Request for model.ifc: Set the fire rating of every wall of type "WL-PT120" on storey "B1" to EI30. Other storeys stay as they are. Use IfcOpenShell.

First a look at what the model holds.

```python
import ifcopenshell
import ifcopenshell.util.element

model = ifcopenshell.open("model.ifc")
print(model.schema)
storey = next(s for s in model.by_type("IfcBuildingStorey") if s.Name == "B1")
walls = [e for e in ifcopenshell.util.element.get_decomposition(storey) if e.is_a("IfcWall")]
seen = {}
for e in walls:
    element_type = ifcopenshell.util.element.get_type(e)
    key = (element_type.Name if element_type != e and element_type else None, ifcopenshell.util.element.get_pset(e, "Pset_WallCommon", "FireRating"))
    seen[key] = seen.get(key, 0) + 1
for (name, value), count in sorted(seen.items(), key=str):
    print(count, "x", name, "|", value)
```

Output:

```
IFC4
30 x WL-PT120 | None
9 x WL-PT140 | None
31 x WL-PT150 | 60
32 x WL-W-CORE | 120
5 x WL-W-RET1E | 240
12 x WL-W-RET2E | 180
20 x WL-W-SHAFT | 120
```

```python
import ifcopenshell
import ifcopenshell.api.pset
import ifcopenshell.util.element

model = ifcopenshell.open("model.ifc")

storey = next(s for s in model.by_type("IfcBuildingStorey") if s.Name == "B1")
walls = [e for e in ifcopenshell.util.element.get_decomposition(storey) if e.is_a("IfcWall")]

count = 0
for e in walls:
    element_type = ifcopenshell.util.element.get_type(e)
    if element_type in (None, e) or element_type.Name != "WL-PT120":
        continue
    # add_pset returns the element's existing set when there is one.
    pset = ifcopenshell.api.pset.add_pset(model, product=e, name="Pset_WallCommon")
    ifcopenshell.api.pset.edit_pset(model, pset=pset, properties={"FireRating": "EI30"})
    count += 1

print(count, "walls updated")

model.write("model_updated.ifc")
```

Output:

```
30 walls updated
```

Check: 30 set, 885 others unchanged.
